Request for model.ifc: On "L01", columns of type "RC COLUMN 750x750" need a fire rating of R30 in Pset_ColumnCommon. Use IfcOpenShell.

First a look at what the model holds.

```python
import ifcopenshell
import ifcopenshell.util.element

model = ifcopenshell.open("model.ifc")
print(model.schema)
storey = next(s for s in model.by_type("IfcBuildingStorey") if s.Name == "L01")
columns = [e for e in ifcopenshell.util.element.get_decomposition(storey) if e.is_a("IfcColumn")]
seen = {}
for e in columns:
    element_type = ifcopenshell.util.element.get_type(e)
    key = (element_type.Name if element_type != e and element_type else None, ifcopenshell.util.element.get_pset(e, "Pset_ColumnCommon", "FireRating"))
    seen[key] = seen.get(key, 0) + 1
for (name, value), count in sorted(seen.items(), key=str):
    print(count, "x", name, "|", value)
```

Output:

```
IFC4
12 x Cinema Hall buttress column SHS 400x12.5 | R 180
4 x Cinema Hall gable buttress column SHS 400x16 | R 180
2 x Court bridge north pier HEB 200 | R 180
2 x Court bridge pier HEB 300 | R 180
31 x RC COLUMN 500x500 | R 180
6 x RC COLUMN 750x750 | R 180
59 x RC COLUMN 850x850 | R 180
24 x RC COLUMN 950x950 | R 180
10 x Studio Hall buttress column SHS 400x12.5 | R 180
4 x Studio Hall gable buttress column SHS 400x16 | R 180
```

```python
import ifcopenshell
import ifcopenshell.api.pset
import ifcopenshell.util.element

model = ifcopenshell.open("model.ifc")

storey = next(s for s in model.by_type("IfcBuildingStorey") if s.Name == "L01")
columns = [e for e in ifcopenshell.util.element.get_decomposition(storey) if e.is_a("IfcColumn")]

count = 0
for e in columns:
    element_type = ifcopenshell.util.element.get_type(e)
    if element_type in (None, e) or element_type.Name != "RC COLUMN 750x750":
        continue
    # add_pset returns the element's existing set when there is one.
    pset = ifcopenshell.api.pset.add_pset(model, product=e, name="Pset_ColumnCommon")
    ifcopenshell.api.pset.edit_pset(model, pset=pset, properties={"FireRating": "R30"})
    count += 1

print(count, "columns updated")

model.write("model_v2.ifc")
```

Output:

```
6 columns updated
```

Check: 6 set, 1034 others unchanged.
